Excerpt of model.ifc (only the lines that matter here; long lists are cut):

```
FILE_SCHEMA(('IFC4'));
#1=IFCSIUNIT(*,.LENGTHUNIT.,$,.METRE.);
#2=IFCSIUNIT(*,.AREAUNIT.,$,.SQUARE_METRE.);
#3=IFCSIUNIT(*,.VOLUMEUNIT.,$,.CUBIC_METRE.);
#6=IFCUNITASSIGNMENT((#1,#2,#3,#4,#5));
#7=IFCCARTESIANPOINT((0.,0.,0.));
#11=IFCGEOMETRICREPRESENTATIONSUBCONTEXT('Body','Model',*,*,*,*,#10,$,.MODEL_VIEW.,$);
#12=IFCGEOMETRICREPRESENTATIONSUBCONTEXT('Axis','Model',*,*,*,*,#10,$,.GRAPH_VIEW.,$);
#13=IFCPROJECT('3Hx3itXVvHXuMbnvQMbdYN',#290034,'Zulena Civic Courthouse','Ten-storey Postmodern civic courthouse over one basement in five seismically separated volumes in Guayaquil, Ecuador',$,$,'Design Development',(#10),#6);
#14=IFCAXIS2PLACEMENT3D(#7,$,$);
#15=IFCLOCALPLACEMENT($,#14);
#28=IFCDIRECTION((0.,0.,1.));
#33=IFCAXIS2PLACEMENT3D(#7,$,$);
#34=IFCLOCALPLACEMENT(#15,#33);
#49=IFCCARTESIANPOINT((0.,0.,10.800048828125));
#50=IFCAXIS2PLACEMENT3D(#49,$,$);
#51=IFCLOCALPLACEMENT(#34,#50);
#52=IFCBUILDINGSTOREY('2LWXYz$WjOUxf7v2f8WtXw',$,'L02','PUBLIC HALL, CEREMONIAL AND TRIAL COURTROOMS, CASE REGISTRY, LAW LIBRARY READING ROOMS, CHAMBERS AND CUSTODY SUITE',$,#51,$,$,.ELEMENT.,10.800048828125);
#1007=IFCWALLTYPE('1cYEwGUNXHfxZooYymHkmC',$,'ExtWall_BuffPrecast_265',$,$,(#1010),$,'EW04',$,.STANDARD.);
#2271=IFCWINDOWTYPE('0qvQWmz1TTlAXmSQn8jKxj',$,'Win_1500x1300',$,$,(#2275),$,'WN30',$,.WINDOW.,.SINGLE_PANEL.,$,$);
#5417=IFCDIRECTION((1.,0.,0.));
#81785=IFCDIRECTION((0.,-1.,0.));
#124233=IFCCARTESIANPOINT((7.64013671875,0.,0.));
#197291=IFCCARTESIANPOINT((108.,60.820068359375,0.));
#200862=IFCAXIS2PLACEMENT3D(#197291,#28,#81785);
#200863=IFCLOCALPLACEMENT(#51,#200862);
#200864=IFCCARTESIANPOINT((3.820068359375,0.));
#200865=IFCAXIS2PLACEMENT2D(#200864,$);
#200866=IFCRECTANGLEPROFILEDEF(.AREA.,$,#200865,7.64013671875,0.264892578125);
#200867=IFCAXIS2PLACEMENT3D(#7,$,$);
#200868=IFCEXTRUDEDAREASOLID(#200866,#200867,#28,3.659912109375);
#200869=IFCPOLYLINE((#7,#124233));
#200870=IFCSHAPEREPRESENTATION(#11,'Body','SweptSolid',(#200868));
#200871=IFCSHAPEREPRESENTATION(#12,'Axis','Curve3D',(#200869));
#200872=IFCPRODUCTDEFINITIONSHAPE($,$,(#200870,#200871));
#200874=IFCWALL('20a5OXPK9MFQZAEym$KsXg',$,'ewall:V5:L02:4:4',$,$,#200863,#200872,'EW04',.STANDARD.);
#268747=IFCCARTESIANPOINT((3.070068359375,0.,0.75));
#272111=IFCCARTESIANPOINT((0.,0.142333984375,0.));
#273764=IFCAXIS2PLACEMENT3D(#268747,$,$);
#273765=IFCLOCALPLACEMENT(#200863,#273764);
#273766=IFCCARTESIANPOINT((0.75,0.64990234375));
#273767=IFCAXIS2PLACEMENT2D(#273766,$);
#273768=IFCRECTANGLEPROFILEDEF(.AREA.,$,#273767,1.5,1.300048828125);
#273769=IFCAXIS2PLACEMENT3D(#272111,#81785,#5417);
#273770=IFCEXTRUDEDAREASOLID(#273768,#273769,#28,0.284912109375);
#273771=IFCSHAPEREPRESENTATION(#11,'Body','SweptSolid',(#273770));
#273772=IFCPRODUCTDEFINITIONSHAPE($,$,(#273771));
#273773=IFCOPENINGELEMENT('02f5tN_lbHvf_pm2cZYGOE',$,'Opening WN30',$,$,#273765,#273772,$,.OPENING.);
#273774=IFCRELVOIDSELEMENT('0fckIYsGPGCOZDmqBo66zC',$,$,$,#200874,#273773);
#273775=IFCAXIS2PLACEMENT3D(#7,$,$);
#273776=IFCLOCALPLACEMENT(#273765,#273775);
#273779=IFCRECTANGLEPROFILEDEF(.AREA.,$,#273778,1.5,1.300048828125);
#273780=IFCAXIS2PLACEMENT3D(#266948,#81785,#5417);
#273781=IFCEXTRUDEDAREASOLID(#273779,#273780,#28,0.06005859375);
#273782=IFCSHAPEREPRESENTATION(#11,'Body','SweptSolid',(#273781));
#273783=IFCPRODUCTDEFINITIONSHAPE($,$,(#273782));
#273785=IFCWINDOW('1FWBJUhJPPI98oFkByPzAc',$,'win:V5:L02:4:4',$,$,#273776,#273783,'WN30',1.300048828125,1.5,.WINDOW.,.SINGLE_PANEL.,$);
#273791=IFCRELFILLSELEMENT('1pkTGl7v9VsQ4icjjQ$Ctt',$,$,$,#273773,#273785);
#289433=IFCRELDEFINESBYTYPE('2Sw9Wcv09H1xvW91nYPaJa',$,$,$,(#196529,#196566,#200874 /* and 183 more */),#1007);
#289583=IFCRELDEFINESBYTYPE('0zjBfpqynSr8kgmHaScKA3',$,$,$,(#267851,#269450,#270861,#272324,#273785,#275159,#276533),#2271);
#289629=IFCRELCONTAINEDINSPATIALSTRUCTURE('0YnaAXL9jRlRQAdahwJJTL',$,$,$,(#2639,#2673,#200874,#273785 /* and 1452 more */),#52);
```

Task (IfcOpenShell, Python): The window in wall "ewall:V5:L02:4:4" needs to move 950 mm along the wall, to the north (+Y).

```python
import ifcopenshell
import ifcopenshell.api.geometry
import ifcopenshell.util.placement

model = ifcopenshell.open("model.ifc")

window = model.by_guid("1FWBJUhJPPI98oFkByPzAc")
opening = window.FillsVoids[0].RelatingOpeningElement
wall = opening.VoidsElements[0].RelatingBuildingElement

wall_matrix = ifcopenshell.util.placement.get_local_placement(wall.ObjectPlacement)
shift = wall_matrix[:3, 0] * -0.95
before = ifcopenshell.util.placement.get_local_placement(window.ObjectPlacement)[:3, 3].copy()

# The window is placed relative to its opening, so it follows when the opening moves.
matrix = ifcopenshell.util.placement.get_local_placement(opening.ObjectPlacement)
matrix[:3, 3] += shift
ifcopenshell.api.geometry.edit_object_placement(
    model, product=opening, matrix=matrix, is_si=False, should_transform_children=True
)

after = ifcopenshell.util.placement.get_local_placement(window.ObjectPlacement)[:3, 3]
print("window moved by", (after - before).round(3) + 0.0)

model.write("model_edited.ifc")
```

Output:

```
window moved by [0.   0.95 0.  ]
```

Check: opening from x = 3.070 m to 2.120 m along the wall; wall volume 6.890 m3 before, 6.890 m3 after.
